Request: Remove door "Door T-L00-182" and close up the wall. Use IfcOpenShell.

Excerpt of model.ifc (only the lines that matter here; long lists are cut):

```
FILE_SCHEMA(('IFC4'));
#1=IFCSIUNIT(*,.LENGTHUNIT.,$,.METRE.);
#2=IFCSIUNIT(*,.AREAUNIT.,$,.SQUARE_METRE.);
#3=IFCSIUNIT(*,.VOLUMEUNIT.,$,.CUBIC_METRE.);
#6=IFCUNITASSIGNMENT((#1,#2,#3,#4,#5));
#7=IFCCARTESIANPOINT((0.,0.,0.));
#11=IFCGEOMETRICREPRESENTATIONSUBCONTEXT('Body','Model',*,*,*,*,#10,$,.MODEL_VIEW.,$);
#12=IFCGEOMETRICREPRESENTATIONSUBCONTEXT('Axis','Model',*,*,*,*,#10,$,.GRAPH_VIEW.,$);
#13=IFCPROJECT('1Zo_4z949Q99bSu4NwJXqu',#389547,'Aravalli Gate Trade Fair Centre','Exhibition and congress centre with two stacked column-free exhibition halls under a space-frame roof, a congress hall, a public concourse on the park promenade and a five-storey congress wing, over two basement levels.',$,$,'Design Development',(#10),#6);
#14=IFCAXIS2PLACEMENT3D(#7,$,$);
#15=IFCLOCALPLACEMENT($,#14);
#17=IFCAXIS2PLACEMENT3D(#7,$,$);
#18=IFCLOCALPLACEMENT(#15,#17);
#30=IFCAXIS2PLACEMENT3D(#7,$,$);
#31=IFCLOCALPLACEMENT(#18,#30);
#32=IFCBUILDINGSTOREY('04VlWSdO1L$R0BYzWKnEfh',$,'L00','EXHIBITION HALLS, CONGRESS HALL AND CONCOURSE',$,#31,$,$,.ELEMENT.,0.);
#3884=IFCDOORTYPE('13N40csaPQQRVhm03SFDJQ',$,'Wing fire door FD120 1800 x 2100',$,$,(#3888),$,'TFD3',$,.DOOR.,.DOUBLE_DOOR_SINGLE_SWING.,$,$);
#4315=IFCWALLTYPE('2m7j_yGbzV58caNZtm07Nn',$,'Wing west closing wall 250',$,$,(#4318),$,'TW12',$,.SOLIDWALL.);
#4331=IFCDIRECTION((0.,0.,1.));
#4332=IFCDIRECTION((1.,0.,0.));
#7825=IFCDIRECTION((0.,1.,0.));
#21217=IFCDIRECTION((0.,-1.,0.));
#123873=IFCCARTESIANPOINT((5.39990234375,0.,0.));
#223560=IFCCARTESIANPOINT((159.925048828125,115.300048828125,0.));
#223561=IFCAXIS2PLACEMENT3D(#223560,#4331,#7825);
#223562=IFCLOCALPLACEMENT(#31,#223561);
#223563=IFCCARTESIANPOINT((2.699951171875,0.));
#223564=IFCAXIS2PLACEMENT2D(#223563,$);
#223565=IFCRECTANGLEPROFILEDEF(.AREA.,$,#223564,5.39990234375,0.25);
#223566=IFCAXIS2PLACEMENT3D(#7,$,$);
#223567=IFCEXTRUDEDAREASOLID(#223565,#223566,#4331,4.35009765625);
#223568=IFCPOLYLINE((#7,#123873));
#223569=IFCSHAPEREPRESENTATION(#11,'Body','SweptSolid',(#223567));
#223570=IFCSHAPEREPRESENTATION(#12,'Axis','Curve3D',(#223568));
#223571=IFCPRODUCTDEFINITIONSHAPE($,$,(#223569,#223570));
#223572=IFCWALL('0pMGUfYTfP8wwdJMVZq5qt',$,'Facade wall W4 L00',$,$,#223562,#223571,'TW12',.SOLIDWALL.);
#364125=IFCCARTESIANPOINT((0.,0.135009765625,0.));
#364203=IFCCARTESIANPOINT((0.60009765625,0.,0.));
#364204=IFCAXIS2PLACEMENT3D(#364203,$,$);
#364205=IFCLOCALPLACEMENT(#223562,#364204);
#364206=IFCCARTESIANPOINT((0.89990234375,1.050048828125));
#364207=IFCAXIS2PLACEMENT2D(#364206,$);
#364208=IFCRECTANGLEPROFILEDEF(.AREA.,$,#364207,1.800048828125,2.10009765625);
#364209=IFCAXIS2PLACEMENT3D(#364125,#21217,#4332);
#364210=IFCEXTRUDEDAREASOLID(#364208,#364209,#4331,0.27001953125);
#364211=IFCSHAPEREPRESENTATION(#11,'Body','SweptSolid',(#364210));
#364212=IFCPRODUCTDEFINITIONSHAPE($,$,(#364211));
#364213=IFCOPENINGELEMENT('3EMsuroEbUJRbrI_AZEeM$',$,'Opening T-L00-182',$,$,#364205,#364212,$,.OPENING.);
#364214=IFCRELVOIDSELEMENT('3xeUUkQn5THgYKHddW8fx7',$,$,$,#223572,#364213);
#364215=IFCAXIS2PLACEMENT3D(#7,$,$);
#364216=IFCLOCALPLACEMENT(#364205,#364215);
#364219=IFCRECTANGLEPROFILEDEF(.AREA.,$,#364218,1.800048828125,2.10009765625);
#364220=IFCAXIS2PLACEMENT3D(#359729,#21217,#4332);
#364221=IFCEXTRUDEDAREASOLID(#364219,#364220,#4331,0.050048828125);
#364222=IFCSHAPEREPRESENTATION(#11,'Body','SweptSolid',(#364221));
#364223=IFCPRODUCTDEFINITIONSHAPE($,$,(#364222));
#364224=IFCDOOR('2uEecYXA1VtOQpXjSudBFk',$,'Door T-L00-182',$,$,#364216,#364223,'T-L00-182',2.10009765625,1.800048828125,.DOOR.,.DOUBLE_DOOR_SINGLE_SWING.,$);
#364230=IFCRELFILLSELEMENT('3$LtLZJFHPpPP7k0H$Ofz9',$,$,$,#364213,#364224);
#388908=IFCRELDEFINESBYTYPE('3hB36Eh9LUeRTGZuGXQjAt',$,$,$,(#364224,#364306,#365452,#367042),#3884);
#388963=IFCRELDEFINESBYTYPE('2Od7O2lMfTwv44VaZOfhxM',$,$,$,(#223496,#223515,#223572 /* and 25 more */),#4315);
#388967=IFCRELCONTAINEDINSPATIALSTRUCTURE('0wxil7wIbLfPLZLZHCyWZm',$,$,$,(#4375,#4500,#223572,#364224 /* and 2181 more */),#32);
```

```python
import ifcopenshell
import ifcopenshell.api.feature
import ifcopenshell.api.root
import ifcopenshell.geom
import ifcopenshell.util.shape

model = ifcopenshell.open("model.ifc")
settings = ifcopenshell.geom.settings()


def volume(element):
    """Net volume in cubic metres, openings subtracted."""
    shape = ifcopenshell.geom.create_shape(settings, element)
    return ifcopenshell.util.shape.get_volume(shape.geometry)


door = model.by_guid("2uEecYXA1VtOQpXjSudBFk")
opening = door.FillsVoids[0].RelatingOpeningElement
wall = opening.VoidsElements[0].RelatingBuildingElement
before = volume(wall)

ifcopenshell.api.root.remove_product(model, product=door)
ifcopenshell.api.feature.remove_feature(model, feature=opening)

after = volume(wall)

print(f"wall volume {before:.3f} -> {after:.3f} m3")

model.write("model-out.ifc")
```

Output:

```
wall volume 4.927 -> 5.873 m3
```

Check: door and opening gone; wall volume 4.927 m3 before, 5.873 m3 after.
